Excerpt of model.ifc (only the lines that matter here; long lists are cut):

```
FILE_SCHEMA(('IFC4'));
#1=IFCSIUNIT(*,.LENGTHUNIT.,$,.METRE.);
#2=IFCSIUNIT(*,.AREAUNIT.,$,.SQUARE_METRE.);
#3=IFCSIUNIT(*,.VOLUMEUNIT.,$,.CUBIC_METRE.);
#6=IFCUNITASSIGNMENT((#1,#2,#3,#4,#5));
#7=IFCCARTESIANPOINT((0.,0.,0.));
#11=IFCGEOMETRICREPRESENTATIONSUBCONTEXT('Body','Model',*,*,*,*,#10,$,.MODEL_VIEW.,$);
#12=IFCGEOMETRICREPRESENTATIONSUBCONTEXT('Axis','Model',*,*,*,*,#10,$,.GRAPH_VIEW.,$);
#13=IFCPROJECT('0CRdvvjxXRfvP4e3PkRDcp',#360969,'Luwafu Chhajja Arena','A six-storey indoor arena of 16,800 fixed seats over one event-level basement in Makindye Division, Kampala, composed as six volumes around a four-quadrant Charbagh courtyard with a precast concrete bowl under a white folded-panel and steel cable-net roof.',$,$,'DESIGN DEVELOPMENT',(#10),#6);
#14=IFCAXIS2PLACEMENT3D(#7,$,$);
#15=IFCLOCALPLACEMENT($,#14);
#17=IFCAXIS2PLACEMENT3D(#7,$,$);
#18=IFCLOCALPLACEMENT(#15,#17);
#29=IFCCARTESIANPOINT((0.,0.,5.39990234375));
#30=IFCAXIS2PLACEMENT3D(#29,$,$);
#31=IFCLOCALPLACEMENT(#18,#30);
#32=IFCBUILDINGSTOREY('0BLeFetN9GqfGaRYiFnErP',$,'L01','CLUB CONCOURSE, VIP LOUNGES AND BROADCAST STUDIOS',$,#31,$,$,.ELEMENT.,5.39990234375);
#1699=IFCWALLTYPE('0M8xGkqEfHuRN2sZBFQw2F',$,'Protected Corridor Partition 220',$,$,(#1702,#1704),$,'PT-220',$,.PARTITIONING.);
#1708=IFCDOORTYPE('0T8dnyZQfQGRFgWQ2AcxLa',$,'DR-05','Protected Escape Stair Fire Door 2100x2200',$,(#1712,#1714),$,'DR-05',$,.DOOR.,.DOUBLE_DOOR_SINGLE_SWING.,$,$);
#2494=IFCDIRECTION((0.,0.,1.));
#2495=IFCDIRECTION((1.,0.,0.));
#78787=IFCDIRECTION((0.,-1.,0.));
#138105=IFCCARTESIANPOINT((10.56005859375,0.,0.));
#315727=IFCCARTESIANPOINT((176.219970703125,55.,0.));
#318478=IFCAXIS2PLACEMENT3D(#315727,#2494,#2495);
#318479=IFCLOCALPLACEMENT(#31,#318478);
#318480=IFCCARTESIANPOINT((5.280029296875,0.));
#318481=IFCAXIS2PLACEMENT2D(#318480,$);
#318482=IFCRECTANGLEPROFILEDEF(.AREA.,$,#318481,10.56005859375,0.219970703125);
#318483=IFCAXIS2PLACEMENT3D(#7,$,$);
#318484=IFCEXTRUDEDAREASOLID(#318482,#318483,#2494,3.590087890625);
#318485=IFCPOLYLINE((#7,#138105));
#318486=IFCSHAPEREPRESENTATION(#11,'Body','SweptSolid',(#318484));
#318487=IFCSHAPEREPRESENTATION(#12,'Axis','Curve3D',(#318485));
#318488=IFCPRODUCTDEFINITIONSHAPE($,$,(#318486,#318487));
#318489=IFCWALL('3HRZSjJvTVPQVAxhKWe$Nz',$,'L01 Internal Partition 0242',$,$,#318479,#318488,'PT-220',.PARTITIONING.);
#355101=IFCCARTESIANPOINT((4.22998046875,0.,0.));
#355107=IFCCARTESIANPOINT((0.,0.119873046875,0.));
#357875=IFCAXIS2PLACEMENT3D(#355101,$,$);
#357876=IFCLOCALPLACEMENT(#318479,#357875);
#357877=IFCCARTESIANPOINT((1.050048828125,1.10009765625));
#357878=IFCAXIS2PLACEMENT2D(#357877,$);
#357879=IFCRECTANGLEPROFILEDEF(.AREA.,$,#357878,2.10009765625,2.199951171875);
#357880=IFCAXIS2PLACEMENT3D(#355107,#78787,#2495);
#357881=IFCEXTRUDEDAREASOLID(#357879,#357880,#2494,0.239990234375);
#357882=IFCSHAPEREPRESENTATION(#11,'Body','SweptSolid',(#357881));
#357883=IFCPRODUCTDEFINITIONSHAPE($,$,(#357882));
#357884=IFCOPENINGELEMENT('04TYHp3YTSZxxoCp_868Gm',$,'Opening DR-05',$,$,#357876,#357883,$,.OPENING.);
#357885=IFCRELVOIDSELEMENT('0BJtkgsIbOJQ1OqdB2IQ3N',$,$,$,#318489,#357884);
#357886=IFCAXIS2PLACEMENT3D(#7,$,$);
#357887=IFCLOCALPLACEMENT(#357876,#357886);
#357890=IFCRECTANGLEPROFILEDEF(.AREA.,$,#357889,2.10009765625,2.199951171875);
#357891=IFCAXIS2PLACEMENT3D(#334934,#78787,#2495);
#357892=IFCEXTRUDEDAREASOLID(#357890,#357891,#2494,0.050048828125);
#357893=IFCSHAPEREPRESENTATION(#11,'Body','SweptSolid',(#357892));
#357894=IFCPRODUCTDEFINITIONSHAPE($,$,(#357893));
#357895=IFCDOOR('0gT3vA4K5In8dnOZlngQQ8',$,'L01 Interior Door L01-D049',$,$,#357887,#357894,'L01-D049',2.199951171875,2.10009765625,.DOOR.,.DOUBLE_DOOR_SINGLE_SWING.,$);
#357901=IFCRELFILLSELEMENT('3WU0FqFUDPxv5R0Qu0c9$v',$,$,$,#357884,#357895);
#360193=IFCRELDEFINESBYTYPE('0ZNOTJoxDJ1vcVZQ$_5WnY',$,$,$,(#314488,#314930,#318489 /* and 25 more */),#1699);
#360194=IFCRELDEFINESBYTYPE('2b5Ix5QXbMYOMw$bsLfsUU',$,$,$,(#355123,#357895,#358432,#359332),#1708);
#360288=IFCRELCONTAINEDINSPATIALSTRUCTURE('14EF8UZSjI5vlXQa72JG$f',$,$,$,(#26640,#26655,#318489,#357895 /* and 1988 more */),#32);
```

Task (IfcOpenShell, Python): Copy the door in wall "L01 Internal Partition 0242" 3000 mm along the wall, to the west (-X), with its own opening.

```python
import ifcopenshell
import ifcopenshell.api.feature
import ifcopenshell.api.geometry
import ifcopenshell.api.root
import ifcopenshell.geom
import ifcopenshell.util.element
import ifcopenshell.util.placement
import ifcopenshell.util.shape

model = ifcopenshell.open("model.ifc")
settings = ifcopenshell.geom.settings()


def volume(element):
    """Net volume in cubic metres, openings subtracted."""
    shape = ifcopenshell.geom.create_shape(settings, element)
    return ifcopenshell.util.shape.get_volume(shape.geometry)


door = model.by_guid("0gT3vA4K5In8dnOZlngQQ8")
opening = door.FillsVoids[0].RelatingOpeningElement
wall = opening.VoidsElements[0].RelatingBuildingElement
before = volume(wall)
shift = ifcopenshell.util.placement.get_local_placement(wall.ObjectPlacement)[:3, 0] * -3.0

# copy_class copies the void relationship, type, container and properties, but no geometry.
new_opening = ifcopenshell.api.root.copy_class(model, product=opening)
new_opening.Representation = ifcopenshell.util.element.copy_deep(
    model, opening.Representation, exclude=["IfcGeometricRepresentationContext", "IfcRepresentationMap"]
)
new_door = ifcopenshell.api.root.copy_class(model, product=door)
new_door.Representation = ifcopenshell.util.element.copy_deep(
    model, door.Representation, exclude=["IfcGeometricRepresentationContext", "IfcRepresentationMap"]
)
new_door.Tag = None
ifcopenshell.api.feature.add_filling(model, opening=new_opening, element=new_door)

for old, new in ((opening, new_opening), (door, new_door)):
    matrix = ifcopenshell.util.placement.get_local_placement(old.ObjectPlacement)
    matrix[:3, 3] += shift
    ifcopenshell.api.geometry.edit_object_placement(model, product=new, matrix=matrix, is_si=False)

after = volume(wall)

print(f"wall volume {before:.3f} -> {after:.3f} m3")

model.write("model_edited.ifc")
```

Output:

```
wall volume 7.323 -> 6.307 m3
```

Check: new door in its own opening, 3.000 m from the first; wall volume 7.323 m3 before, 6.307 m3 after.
